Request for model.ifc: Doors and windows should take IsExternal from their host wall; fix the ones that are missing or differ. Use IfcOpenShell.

First a look at what the model holds.

```python
import ifcopenshell
import ifcopenshell.util.element

model = ifcopenshell.open("model.ifc")
print(model.schema)
seen = {}
for e in model.by_type("IfcDoor") + model.by_type("IfcWindow"):
    if not e.FillsVoids:
        continue
    host = e.FillsVoids[0].RelatingOpeningElement.VoidsElements[0].RelatingBuildingElement
    own = ifcopenshell.util.element.get_pset(e, f"Pset_{e.is_a()[3:].removesuffix('StandardCase')}Common", "IsExternal")
    wall = ifcopenshell.util.element.get_pset(host, "Pset_WallCommon", "IsExternal")
    seen[e.is_a(), own, wall] = seen.get((e.is_a(), own, wall), 0) + 1
for (cls, own, wall), count in sorted(seen.items(), key=str):
    print(count, cls, "IsExternal:", own, "| host wall:", wall)
```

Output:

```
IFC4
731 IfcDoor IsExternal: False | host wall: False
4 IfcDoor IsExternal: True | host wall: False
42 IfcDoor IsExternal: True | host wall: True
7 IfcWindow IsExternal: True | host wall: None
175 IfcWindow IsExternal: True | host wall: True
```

```python
import ifcopenshell
import ifcopenshell.api.pset
import ifcopenshell.util.element

model = ifcopenshell.open("model.ifc")

count = 0
for ifc_class, pset_name in (("IfcDoor", "Pset_DoorCommon"), ("IfcWindow", "Pset_WindowCommon")):
    for e in model.by_type(ifc_class):
        if not e.FillsVoids:
            continue
        host = e.FillsVoids[0].RelatingOpeningElement.VoidsElements[0].RelatingBuildingElement
        external = ifcopenshell.util.element.get_pset(host, "Pset_WallCommon", "IsExternal")
        if external is None or ifcopenshell.util.element.get_pset(e, pset_name, "IsExternal") == external:
            continue
        pset = ifcopenshell.api.pset.add_pset(model, product=e, name=pset_name)
        ifcopenshell.api.pset.edit_pset(model, pset=pset, properties={"IsExternal": external})
        count += 1

print(count, "updated")

model.write("model_edited.ifc")
```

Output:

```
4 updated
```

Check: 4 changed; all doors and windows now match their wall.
